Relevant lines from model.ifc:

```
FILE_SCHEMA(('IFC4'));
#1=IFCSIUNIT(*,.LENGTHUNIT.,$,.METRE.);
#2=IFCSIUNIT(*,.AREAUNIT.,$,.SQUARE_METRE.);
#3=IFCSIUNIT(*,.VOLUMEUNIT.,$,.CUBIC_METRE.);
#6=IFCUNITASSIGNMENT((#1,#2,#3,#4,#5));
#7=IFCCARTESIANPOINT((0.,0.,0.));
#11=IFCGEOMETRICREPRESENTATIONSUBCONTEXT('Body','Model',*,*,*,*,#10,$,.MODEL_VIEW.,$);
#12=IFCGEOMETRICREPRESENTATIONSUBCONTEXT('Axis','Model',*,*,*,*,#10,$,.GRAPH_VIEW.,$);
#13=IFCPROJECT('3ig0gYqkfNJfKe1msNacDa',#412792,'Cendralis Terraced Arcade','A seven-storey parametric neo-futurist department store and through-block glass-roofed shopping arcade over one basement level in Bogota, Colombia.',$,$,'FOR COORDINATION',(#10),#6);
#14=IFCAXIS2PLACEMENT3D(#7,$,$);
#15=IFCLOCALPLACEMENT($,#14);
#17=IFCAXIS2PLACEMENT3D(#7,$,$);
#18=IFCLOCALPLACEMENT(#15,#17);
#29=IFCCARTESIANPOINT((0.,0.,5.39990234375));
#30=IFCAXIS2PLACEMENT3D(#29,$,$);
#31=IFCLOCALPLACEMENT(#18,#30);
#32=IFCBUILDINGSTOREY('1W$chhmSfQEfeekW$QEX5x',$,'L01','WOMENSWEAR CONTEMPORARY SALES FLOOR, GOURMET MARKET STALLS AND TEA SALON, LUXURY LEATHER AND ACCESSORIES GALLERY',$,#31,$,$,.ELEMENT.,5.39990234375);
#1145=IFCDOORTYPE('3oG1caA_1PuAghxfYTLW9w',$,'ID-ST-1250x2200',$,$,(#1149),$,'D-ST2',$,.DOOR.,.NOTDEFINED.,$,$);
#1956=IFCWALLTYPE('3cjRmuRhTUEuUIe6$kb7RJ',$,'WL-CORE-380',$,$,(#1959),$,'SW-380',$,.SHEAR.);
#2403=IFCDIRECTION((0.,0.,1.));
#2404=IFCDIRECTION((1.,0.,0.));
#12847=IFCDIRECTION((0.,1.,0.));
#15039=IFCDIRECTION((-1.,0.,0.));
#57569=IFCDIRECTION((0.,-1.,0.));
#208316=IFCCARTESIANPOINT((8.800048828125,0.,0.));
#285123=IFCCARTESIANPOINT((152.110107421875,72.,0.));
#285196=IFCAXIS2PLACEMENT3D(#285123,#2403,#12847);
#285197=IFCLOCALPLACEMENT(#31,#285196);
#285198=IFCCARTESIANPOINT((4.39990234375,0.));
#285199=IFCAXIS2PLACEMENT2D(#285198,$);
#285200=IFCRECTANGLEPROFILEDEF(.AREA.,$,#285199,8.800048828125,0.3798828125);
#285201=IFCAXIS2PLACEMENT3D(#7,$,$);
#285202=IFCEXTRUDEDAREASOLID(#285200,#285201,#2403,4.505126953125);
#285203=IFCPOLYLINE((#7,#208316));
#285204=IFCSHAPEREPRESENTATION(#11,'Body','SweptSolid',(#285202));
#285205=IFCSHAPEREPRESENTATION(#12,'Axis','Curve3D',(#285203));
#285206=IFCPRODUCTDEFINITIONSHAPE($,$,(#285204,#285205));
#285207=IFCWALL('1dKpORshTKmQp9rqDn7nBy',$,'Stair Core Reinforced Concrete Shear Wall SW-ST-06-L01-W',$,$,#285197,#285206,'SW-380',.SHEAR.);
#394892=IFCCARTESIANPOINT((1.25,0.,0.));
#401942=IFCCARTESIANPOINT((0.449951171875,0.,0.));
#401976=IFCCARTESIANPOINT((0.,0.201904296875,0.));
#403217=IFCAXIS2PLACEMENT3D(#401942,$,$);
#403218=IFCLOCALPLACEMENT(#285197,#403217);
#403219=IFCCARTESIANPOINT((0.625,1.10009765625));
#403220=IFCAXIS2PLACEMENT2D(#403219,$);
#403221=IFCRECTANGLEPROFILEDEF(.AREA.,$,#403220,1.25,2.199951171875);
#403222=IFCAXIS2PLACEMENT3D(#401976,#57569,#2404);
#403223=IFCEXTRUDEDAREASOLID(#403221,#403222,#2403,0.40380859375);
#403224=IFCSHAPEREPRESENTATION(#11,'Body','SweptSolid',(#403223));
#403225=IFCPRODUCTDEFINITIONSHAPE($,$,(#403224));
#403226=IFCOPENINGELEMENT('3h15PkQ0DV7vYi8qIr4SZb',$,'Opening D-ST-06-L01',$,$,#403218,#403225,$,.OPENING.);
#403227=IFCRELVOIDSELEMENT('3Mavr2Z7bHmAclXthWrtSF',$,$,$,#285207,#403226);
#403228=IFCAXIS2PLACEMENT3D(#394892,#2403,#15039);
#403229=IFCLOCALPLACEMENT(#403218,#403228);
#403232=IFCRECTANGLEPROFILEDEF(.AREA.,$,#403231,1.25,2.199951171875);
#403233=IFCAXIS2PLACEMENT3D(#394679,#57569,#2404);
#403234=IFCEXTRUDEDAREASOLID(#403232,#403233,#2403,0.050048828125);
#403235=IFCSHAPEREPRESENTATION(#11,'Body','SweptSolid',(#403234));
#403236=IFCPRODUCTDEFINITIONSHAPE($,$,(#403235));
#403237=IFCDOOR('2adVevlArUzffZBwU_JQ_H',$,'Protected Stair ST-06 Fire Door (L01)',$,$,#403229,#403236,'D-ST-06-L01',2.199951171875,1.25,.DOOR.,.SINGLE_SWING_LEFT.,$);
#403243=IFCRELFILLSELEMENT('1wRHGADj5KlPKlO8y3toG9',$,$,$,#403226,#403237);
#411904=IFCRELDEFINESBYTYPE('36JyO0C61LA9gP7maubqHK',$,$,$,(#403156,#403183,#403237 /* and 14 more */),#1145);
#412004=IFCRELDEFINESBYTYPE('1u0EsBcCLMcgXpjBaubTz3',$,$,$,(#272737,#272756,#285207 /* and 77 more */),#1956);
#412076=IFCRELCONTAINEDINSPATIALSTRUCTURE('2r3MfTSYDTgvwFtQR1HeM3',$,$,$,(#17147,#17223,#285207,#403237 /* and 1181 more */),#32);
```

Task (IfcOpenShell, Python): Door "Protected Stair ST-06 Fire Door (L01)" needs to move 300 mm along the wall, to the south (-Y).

```python
import ifcopenshell
import ifcopenshell.api.geometry
import ifcopenshell.util.placement
import ifcopenshell.util.unit

model = ifcopenshell.open("model.ifc")
unit_scale = ifcopenshell.util.unit.calculate_unit_scale(model)

door = model.by_guid("2adVevlArUzffZBwU_JQ_H")
opening = door.FillsVoids[0].RelatingOpeningElement
wall = opening.VoidsElements[0].RelatingBuildingElement

wall_matrix = ifcopenshell.util.placement.get_local_placement(wall.ObjectPlacement)
shift = wall_matrix[:3, 0] * -0.3 / unit_scale
before = ifcopenshell.util.placement.get_local_placement(door.ObjectPlacement)[:3, 3].copy()

# The door is placed relative to its opening, so it follows when the opening moves.
matrix = ifcopenshell.util.placement.get_local_placement(opening.ObjectPlacement)
matrix[:3, 3] += shift
ifcopenshell.api.geometry.edit_object_placement(
    model, product=opening, matrix=matrix, is_si=False, should_transform_children=True
)

after = ifcopenshell.util.placement.get_local_placement(door.ObjectPlacement)[:3, 3]
print("door moved by", (after - before).round(3) + 0.0)

model.write("model_updated.ifc")
```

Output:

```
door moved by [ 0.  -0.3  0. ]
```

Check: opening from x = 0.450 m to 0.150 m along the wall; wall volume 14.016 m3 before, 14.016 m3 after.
